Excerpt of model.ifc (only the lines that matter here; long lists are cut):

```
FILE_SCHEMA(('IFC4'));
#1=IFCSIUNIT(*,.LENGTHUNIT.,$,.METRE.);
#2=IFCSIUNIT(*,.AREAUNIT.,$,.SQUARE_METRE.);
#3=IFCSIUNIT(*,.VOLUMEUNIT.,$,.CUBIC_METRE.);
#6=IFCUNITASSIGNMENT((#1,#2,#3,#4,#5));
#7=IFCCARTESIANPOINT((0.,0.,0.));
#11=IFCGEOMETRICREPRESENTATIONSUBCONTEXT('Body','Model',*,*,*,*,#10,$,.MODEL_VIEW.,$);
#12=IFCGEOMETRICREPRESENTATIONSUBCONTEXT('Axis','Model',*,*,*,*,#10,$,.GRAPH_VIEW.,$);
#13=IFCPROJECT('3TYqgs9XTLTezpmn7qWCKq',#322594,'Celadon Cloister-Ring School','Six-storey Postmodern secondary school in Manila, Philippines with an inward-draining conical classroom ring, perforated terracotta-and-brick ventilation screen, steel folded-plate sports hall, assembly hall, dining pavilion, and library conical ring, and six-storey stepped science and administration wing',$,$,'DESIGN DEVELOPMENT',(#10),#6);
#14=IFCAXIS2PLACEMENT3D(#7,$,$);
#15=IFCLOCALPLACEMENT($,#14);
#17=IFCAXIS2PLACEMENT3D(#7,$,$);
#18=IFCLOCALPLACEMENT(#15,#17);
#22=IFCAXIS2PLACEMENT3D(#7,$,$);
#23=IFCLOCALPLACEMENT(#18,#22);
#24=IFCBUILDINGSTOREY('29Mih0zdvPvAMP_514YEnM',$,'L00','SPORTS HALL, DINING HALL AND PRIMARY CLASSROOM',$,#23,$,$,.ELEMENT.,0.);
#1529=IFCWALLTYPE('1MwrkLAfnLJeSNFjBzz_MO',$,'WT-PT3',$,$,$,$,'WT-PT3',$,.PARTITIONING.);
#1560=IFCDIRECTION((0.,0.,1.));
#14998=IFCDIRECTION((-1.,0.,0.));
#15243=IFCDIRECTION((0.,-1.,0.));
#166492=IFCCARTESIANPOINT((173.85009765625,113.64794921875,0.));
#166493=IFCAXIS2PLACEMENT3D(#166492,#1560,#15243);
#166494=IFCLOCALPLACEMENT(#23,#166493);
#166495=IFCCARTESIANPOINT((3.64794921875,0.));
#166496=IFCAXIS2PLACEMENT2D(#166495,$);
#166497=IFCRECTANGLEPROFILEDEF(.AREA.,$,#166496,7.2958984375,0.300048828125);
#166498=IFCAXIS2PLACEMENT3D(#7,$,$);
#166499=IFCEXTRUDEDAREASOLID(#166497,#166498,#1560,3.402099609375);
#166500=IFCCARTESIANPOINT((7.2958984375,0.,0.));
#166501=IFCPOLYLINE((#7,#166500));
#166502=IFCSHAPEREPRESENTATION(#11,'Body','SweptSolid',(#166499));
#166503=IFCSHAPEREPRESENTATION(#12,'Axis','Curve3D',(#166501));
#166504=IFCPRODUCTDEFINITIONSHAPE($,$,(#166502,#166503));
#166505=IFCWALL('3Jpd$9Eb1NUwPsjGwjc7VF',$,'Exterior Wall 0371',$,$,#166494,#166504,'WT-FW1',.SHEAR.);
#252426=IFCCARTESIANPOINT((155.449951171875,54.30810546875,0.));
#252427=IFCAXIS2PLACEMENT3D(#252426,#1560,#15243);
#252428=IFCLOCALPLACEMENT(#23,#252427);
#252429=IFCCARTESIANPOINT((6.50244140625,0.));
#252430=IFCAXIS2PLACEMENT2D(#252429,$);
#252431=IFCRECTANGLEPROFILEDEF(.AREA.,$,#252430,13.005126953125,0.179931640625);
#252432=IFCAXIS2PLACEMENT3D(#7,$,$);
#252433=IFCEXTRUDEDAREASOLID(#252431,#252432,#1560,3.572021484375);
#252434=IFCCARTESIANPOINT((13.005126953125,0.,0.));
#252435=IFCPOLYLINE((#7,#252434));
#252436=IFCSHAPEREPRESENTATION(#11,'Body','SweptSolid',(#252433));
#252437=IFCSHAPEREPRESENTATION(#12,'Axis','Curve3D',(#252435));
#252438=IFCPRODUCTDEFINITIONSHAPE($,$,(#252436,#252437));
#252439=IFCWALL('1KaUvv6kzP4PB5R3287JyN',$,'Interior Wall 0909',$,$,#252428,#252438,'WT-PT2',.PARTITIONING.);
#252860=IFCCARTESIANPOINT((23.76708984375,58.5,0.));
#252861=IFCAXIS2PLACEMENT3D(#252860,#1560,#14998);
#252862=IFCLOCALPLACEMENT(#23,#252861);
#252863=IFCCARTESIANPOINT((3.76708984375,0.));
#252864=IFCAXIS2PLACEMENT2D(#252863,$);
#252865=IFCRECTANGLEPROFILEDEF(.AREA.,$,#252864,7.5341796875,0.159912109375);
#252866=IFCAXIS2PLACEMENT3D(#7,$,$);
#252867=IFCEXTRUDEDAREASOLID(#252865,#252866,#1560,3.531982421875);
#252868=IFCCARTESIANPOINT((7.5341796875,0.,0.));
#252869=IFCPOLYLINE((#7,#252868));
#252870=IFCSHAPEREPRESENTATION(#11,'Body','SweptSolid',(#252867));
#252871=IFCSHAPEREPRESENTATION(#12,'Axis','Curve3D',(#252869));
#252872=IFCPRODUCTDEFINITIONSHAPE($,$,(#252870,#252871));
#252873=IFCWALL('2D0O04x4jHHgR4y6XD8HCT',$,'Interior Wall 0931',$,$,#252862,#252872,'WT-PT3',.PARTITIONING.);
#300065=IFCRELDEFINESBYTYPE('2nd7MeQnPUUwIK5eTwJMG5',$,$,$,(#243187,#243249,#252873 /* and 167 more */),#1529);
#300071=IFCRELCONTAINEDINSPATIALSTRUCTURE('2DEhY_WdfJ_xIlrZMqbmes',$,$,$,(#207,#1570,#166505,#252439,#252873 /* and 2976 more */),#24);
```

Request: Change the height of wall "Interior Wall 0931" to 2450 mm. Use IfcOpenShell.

```python
import ifcopenshell
import ifcopenshell.geom
import ifcopenshell.util.representation
import ifcopenshell.util.shape

model = ifcopenshell.open("model.ifc")
settings = ifcopenshell.geom.settings()


def volume(element):
    """Net volume in cubic metres, openings subtracted."""
    shape = ifcopenshell.geom.create_shape(settings, element)
    return ifcopenshell.util.shape.get_volume(shape.geometry)


wall = model.by_guid("2D0O04x4jHHgR4y6XD8HCT")
before = volume(wall)

body = ifcopenshell.util.representation.get_representation(wall, "Model", "Body")
solid = body.Items[0]
old_height = solid.Depth
solid.Depth = 2.45
after = volume(wall)

print(f"height {old_height:g} -> {solid.Depth:g}, volume {before:.3f} -> {after:.3f} m3")

model.write("model_updated.ifc")
```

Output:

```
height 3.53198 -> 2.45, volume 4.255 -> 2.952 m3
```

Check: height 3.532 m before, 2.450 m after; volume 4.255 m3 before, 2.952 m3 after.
